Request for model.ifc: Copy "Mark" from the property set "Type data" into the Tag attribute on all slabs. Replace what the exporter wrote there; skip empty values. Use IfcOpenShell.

First a look at what the model holds.

```python
import ifcopenshell
import ifcopenshell.util.element

model = ifcopenshell.open("model.ifc")
print(model.schema)
slabs = model.by_type("IfcSlab")
print(len(slabs), "slabs")
for e in slabs[:8]:
    source = ifcopenshell.util.element.get_pset(e, "Type data", "Mark")
    target = e.Tag
    print(e.id(), repr(source), repr(target), sep=" | ")
```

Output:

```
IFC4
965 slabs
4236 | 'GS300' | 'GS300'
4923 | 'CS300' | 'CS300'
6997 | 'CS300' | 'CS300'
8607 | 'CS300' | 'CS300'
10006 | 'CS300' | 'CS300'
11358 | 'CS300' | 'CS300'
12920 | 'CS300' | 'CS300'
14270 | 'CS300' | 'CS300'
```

```python
import ifcopenshell
import ifcopenshell.util.element

model = ifcopenshell.open("model.ifc")

count = 0
for e in model.by_type("IfcSlab"):
    value = ifcopenshell.util.element.get_pset(e, "Type data", "Mark")
    current = e.Tag
    if not value or not value.strip() or current == value:
        continue
    e.Tag = value
    count += 1

print(count, "slabs updated")

model.write("model_edited.ifc")
```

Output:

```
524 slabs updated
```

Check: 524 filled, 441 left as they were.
